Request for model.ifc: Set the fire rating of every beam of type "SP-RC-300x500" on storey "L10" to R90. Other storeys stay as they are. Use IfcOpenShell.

First a look at what the model holds.

```python
import ifcopenshell
import ifcopenshell.util.element

model = ifcopenshell.open("model.ifc")
print(model.schema)
storey = next(s for s in model.by_type("IfcBuildingStorey") if s.Name == "L10")
beams = [e for e in ifcopenshell.util.element.get_decomposition(storey) if e.is_a("IfcBeam")]
seen = {}
for e in beams:
    element_type = ifcopenshell.util.element.get_type(e)
    key = (element_type.Name if element_type != e and element_type else None, ifcopenshell.util.element.get_pset(e, "Pset_BeamCommon", "FireRating"))
    seen[key] = seen.get(key, 0) + 1
for (name, value), count in sorted(seen.items(), key=str):
    print(count, "x", name, "|", value)
```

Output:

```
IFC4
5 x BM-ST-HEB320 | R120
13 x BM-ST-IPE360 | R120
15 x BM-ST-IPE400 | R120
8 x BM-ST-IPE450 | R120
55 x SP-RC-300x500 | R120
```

```python
import ifcopenshell
import ifcopenshell.api.pset
import ifcopenshell.util.element

model = ifcopenshell.open("model.ifc")

storey = next(s for s in model.by_type("IfcBuildingStorey") if s.Name == "L10")
beams = [e for e in ifcopenshell.util.element.get_decomposition(storey) if e.is_a("IfcBeam")]

count = 0
for e in beams:
    element_type = ifcopenshell.util.element.get_type(e)
    if element_type in (None, e) or element_type.Name != "SP-RC-300x500":
        continue
    # add_pset returns the element's existing set when there is one.
    pset = ifcopenshell.api.pset.add_pset(model, product=e, name="Pset_BeamCommon")
    ifcopenshell.api.pset.edit_pset(model, pset=pset, properties={"FireRating": "R90"})
    count += 1

print(count, "beams updated")

model.write("model_edited.ifc")
```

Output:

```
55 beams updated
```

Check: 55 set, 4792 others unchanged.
